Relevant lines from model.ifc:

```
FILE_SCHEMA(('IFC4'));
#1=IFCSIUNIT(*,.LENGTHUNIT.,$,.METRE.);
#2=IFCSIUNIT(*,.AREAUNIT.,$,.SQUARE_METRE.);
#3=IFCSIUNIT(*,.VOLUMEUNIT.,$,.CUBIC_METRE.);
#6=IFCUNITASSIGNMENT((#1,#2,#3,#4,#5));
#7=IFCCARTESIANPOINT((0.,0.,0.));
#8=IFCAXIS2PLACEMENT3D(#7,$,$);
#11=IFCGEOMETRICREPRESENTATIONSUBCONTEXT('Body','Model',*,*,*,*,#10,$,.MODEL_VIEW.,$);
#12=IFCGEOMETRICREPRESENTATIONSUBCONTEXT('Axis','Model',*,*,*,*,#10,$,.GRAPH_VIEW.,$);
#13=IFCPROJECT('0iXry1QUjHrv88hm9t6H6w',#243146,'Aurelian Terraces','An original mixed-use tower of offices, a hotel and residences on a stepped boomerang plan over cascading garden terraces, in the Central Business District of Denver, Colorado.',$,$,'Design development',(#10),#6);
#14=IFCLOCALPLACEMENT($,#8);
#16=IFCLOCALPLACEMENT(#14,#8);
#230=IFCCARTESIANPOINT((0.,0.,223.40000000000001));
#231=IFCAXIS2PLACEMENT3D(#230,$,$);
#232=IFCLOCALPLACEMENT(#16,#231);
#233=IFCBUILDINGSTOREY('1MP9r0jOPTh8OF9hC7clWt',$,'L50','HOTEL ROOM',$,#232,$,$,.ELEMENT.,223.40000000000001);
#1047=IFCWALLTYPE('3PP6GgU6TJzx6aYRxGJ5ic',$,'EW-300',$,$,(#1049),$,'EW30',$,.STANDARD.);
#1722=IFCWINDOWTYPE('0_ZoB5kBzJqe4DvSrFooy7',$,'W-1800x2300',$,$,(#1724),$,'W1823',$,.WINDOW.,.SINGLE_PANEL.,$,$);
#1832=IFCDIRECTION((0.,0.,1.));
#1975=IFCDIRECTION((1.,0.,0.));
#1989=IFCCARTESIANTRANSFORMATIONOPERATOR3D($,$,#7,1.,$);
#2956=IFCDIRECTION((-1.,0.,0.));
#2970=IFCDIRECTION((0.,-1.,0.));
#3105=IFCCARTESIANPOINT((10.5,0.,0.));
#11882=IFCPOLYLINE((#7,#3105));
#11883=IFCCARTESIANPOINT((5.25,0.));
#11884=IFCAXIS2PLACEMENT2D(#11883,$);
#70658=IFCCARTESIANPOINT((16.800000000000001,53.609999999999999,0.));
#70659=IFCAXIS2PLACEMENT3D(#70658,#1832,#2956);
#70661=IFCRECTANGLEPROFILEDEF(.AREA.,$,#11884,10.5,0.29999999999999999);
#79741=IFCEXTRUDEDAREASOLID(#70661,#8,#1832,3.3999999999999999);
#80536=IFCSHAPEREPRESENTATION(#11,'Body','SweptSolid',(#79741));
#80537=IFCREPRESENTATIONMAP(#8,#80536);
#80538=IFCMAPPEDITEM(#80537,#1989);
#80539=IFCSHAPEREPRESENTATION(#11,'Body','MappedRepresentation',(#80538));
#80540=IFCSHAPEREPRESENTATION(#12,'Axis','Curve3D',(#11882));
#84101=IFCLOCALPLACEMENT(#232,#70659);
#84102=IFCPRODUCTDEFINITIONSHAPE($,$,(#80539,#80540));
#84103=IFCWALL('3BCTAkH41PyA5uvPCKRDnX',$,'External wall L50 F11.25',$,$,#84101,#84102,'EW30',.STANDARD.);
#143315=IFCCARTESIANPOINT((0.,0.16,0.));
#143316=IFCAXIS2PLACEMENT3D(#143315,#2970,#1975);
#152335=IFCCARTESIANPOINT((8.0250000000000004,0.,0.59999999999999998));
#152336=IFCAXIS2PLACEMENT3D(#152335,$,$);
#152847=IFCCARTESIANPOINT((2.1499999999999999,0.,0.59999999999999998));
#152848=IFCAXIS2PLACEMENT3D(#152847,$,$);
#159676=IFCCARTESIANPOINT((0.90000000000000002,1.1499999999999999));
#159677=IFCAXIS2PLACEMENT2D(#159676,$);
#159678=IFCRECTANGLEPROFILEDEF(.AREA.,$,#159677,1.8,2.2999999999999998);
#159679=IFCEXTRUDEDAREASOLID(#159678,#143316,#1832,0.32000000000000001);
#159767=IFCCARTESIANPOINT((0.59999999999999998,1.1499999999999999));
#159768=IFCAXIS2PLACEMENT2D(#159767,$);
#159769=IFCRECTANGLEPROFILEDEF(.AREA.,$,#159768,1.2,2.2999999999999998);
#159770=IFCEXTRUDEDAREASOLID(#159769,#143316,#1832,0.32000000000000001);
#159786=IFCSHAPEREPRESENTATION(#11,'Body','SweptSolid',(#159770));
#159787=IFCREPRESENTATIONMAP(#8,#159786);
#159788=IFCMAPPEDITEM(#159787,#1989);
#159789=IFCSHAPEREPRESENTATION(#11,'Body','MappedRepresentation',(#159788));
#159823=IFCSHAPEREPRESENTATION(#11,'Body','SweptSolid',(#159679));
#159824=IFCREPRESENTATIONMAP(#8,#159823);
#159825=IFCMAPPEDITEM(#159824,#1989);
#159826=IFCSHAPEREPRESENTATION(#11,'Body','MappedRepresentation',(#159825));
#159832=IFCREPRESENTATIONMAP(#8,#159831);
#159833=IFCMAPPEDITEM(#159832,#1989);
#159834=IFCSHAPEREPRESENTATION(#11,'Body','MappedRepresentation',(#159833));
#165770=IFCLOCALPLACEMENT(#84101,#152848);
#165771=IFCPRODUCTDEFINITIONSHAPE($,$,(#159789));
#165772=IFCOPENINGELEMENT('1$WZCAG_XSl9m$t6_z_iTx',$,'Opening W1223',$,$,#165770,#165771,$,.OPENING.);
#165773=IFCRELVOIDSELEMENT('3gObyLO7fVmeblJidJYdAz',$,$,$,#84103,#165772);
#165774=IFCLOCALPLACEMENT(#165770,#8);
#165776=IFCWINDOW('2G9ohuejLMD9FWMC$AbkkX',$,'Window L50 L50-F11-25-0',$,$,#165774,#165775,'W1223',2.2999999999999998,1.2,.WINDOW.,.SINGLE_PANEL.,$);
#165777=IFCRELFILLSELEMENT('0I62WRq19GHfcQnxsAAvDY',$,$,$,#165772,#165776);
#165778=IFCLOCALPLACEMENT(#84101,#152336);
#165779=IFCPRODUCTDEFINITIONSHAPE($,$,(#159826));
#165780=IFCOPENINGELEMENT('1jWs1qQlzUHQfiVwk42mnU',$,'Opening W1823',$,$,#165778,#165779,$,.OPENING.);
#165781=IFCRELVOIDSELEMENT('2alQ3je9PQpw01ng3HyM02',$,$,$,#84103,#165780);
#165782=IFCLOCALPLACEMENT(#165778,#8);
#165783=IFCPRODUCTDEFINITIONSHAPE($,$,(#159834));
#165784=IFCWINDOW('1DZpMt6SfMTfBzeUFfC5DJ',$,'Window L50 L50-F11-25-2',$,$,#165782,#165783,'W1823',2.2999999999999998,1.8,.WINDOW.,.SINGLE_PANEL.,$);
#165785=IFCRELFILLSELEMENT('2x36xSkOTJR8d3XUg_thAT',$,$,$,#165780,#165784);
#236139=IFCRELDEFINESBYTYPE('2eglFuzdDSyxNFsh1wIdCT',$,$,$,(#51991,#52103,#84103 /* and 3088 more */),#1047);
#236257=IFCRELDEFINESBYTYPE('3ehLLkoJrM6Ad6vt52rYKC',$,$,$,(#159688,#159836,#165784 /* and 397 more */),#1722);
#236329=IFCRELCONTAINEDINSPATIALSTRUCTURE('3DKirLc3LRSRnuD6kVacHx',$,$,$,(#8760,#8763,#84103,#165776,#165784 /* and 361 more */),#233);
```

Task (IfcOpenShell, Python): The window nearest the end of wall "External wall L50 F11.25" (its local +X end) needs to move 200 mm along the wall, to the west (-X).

```python
import ifcopenshell
import ifcopenshell.api.geometry
import ifcopenshell.util.placement
import ifcopenshell.util.unit

model = ifcopenshell.open("model.ifc")
unit_scale = ifcopenshell.util.unit.calculate_unit_scale(model)

window = model.by_id(165784)
opening = window.FillsVoids[0].RelatingOpeningElement
wall = opening.VoidsElements[0].RelatingBuildingElement

wall_matrix = ifcopenshell.util.placement.get_local_placement(wall.ObjectPlacement)
shift = wall_matrix[:3, 0] * 0.2 / unit_scale
before = ifcopenshell.util.placement.get_local_placement(window.ObjectPlacement)[:3, 3].copy()

# The window is placed relative to its opening, so it follows when the opening moves.
matrix = ifcopenshell.util.placement.get_local_placement(opening.ObjectPlacement)
matrix[:3, 3] += shift
ifcopenshell.api.geometry.edit_object_placement(
    model, product=opening, matrix=matrix, is_si=False, should_transform_children=True
)

after = ifcopenshell.util.placement.get_local_placement(window.ObjectPlacement)[:3, 3]
print("window moved by", (after - before).round(3) + 0.0)

model.write("model_rev.ifc")
```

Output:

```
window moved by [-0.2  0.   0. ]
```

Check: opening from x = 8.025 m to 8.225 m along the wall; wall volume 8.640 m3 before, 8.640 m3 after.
